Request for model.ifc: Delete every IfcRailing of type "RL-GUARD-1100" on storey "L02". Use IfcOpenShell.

First a look at what the model holds.

```python
import ifcopenshell
import ifcopenshell.util.element

model = ifcopenshell.open("model.ifc")
print(model.schema)
storey = next(s for s in model.by_type("IfcBuildingStorey") if s.Name == "L02")
railings = [e for e in ifcopenshell.util.element.get_decomposition(storey) if e.is_a("IfcRailing")]
seen = {}
for e in railings:
    element_type = ifcopenshell.util.element.get_type(e)
    name = element_type.Name if element_type not in (None, e) else None
    seen[name] = seen.get(name, 0) + 1
for name, count in sorted(seen.items(), key=str):
    print(count, "x", name)
```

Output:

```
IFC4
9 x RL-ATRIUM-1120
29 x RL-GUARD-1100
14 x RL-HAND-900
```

```python
import ifcopenshell
import ifcopenshell.api.root
import ifcopenshell.util.element

model = ifcopenshell.open("model.ifc")

storey = next(s for s in model.by_type("IfcBuildingStorey") if s.Name == "L02")
railings = [e for e in ifcopenshell.util.element.get_decomposition(storey) if e.is_a("IfcRailing")]
targets = [e for e in railings if (t := ifcopenshell.util.element.get_type(e)) not in (None, e) and t.Name == "RL-GUARD-1100"]

for e in targets:
    ifcopenshell.api.root.remove_product(model, product=e)
print(len(targets), "removed")

model.write("model-out.ifc")
```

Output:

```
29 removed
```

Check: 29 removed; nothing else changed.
